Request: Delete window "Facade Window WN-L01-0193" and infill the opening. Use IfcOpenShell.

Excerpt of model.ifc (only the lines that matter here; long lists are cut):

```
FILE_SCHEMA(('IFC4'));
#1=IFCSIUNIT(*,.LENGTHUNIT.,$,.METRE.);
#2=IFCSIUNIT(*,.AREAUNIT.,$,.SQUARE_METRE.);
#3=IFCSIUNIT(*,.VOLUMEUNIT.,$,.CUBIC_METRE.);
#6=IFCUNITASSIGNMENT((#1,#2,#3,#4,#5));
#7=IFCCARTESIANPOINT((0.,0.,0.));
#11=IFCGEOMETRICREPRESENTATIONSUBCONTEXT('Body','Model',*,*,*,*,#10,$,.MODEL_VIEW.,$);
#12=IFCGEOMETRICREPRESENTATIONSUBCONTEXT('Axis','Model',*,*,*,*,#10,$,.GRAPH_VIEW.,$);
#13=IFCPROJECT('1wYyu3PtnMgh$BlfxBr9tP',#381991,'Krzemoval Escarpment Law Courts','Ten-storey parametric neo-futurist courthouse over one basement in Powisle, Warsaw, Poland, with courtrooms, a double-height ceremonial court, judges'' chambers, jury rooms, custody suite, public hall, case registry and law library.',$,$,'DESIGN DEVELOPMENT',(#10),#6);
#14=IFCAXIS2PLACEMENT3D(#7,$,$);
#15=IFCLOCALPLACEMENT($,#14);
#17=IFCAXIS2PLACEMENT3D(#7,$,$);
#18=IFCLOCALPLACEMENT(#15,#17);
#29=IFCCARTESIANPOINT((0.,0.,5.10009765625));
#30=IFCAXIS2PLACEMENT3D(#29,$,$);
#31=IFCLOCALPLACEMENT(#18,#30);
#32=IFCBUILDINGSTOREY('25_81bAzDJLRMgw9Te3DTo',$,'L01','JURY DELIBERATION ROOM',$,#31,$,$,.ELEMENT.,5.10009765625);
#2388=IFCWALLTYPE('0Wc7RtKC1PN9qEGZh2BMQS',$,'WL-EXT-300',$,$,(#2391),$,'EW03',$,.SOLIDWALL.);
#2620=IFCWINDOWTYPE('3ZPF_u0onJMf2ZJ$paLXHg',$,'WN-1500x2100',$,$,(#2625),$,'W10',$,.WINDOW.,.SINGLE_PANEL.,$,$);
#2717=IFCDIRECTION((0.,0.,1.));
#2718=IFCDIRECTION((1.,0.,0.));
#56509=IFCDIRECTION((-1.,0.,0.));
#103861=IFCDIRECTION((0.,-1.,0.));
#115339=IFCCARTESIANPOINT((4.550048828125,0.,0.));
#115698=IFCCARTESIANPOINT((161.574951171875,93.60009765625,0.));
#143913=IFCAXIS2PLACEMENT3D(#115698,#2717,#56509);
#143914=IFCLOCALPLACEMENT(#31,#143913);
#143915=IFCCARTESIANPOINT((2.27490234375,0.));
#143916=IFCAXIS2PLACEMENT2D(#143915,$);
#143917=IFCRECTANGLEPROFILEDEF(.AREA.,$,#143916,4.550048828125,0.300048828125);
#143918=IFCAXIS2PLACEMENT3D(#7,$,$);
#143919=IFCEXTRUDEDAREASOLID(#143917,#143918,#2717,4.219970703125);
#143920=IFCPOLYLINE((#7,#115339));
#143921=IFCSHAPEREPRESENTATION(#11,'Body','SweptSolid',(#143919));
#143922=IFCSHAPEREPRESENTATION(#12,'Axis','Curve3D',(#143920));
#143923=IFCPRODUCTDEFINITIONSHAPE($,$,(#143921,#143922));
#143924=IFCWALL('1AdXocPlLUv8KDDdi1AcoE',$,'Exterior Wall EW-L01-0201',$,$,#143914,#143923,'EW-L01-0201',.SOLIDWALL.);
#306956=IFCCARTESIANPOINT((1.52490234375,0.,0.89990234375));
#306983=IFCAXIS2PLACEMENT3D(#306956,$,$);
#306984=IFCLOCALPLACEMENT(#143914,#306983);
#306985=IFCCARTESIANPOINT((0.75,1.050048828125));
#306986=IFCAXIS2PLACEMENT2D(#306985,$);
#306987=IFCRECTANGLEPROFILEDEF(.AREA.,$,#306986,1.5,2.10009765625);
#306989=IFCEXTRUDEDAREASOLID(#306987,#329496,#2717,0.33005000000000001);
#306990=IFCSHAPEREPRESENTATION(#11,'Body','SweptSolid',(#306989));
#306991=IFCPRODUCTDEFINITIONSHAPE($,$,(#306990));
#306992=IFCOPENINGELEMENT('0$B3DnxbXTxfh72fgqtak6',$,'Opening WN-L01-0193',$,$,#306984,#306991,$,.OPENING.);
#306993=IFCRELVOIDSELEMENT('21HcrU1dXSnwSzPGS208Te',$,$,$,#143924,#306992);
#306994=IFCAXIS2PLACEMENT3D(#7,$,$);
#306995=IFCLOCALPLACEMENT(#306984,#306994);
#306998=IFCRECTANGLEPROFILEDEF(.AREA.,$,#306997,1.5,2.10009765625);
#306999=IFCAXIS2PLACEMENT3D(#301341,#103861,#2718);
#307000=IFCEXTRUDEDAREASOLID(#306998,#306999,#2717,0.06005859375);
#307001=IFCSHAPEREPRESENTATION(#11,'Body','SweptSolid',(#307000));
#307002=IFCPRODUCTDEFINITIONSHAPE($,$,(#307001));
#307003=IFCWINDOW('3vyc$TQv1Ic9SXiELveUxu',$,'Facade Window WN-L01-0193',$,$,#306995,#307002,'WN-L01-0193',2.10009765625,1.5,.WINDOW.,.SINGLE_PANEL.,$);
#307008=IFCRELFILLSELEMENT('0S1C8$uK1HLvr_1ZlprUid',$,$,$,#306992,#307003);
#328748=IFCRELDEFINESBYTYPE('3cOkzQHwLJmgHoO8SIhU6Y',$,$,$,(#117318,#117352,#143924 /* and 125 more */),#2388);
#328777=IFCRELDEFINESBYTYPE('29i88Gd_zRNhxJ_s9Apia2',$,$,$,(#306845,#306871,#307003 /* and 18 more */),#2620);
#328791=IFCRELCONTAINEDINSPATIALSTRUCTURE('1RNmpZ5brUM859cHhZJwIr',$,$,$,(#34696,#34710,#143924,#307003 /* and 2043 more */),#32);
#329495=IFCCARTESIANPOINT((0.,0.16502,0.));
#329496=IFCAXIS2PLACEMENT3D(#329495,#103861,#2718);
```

```python
import ifcopenshell
import ifcopenshell.api.feature
import ifcopenshell.api.root
import ifcopenshell.geom
import ifcopenshell.util.shape

model = ifcopenshell.open("model.ifc")
settings = ifcopenshell.geom.settings()


def volume(element):
    """Net volume in cubic metres, openings subtracted."""
    shape = ifcopenshell.geom.create_shape(settings, element)
    return ifcopenshell.util.shape.get_volume(shape.geometry)


window = model.by_guid("3vyc$TQv1Ic9SXiELveUxu")
opening = window.FillsVoids[0].RelatingOpeningElement
wall = opening.VoidsElements[0].RelatingBuildingElement
before = volume(wall)

ifcopenshell.api.root.remove_product(model, product=window)
ifcopenshell.api.feature.remove_feature(model, feature=opening)

after = volume(wall)

print(f"wall volume {before:.3f} -> {after:.3f} m3")

model.write("model_rev.ifc")
```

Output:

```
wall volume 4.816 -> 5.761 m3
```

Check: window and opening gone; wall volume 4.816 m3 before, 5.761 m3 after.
